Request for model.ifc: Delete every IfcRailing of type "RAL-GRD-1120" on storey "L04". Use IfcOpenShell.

First a look at what the model holds.

```python
import ifcopenshell
import ifcopenshell.util.element

model = ifcopenshell.open("model.ifc")
print(model.schema)
storey = next(s for s in model.by_type("IfcBuildingStorey") if s.Name == "L04")
railings = [e for e in ifcopenshell.util.element.get_decomposition(storey) if e.is_a("IfcRailing")]
seen = {}
for e in railings:
    element_type = ifcopenshell.util.element.get_type(e)
    name = element_type.Name if element_type not in (None, e) else None
    seen[name] = seen.get(name, 0) + 1
for name, count in sorted(seen.items(), key=str):
    print(count, "x", name)
```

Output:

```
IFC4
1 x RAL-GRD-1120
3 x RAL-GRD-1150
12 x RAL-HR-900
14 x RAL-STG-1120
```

```python
import ifcopenshell
import ifcopenshell.api.root
import ifcopenshell.util.element

model = ifcopenshell.open("model.ifc")

storey = next(s for s in model.by_type("IfcBuildingStorey") if s.Name == "L04")
railings = [e for e in ifcopenshell.util.element.get_decomposition(storey) if e.is_a("IfcRailing")]
targets = [e for e in railings if (t := ifcopenshell.util.element.get_type(e)) not in (None, e) and t.Name == "RAL-GRD-1120"]

for e in targets:
    ifcopenshell.api.root.remove_product(model, product=e)
print(len(targets), "removed")

model.write("model_edited.ifc")
```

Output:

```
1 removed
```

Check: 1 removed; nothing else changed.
